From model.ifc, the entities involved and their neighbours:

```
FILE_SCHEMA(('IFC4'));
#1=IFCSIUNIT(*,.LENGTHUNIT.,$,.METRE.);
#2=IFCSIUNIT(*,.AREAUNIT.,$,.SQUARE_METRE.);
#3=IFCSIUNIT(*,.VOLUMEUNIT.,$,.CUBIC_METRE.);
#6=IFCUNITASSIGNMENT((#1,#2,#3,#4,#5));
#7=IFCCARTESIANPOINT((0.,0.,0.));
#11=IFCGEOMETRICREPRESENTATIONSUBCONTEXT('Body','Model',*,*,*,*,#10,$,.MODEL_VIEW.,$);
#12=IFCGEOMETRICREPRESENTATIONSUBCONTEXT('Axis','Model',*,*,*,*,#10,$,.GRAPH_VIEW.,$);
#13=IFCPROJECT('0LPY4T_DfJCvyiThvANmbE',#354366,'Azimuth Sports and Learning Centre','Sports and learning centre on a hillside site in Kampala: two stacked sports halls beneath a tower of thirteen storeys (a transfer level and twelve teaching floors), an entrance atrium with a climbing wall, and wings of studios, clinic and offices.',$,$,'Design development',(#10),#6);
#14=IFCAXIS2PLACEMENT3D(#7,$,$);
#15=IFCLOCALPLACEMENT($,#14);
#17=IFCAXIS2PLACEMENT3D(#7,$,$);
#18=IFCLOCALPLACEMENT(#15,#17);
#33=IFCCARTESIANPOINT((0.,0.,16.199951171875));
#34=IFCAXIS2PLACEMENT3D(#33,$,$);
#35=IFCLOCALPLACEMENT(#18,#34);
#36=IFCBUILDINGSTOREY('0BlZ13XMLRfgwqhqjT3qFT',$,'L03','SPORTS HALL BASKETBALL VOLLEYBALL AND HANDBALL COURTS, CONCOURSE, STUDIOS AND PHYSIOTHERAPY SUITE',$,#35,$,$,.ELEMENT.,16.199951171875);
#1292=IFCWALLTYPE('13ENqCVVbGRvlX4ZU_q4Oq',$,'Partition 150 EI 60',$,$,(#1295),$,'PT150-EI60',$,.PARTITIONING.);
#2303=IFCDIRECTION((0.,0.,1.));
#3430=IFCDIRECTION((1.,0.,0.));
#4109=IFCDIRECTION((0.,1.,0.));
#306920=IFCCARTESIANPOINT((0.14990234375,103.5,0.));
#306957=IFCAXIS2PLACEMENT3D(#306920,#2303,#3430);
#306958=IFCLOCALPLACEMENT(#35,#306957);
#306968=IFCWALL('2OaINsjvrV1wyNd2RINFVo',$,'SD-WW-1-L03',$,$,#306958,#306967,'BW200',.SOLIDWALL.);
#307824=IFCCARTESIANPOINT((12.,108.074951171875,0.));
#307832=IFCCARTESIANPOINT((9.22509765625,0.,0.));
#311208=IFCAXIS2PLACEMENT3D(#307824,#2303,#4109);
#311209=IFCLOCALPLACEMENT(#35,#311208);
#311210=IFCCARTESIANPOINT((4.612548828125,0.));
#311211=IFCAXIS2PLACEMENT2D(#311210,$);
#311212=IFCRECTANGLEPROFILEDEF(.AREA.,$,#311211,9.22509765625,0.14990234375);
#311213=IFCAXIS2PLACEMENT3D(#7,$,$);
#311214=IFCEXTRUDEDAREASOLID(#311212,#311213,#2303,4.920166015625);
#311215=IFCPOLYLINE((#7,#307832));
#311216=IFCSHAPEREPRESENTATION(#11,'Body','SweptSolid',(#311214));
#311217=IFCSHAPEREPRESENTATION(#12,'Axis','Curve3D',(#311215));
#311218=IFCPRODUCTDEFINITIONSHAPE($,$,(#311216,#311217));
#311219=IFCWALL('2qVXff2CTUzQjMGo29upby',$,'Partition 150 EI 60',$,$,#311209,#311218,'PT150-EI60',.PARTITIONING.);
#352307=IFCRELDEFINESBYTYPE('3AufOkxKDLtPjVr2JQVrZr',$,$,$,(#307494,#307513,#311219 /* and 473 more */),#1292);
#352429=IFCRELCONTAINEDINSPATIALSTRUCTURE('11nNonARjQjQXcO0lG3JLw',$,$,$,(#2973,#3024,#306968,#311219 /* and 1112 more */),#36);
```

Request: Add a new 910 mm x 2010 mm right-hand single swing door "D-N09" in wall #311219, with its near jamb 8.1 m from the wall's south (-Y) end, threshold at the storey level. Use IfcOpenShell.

```python
import numpy as np
import ifcopenshell
import ifcopenshell.api.feature
import ifcopenshell.api.geometry
import ifcopenshell.api.root
import ifcopenshell.api.spatial
import ifcopenshell.geom
import ifcopenshell.util.element
import ifcopenshell.util.placement
import ifcopenshell.util.representation
import ifcopenshell.util.shape
import ifcopenshell.util.unit

model = ifcopenshell.open("model.ifc")
unit_scale = ifcopenshell.util.unit.calculate_unit_scale(model)
settings = ifcopenshell.geom.settings()


def volume(element):
    """Net volume in cubic metres, openings subtracted."""
    shape = ifcopenshell.geom.create_shape(settings, element)
    return ifcopenshell.util.shape.get_volume(shape.geometry)


wall = model.by_id(311219)
storey = ifcopenshell.util.element.get_container(wall, ifc_class="IfcBuildingStorey")
context = ifcopenshell.util.representation.get_context(model, "Model", "Body", "MODEL_VIEW")
before = volume(wall)

width, height, from_end, sill = 0.91, 2.01, 8.1, 0.0  # metres

# The wall runs along its own X axis, and the end named is its -X end.
wall_shape = ifcopenshell.geom.create_shape(settings, wall)
x, y, z = ifcopenshell.util.shape.get_vertices(wall_shape.geometry).T
start = x.min() + from_end
face, thickness = float(y.min()), float(y.max() - y.min())
wall_matrix = ifcopenshell.util.placement.get_local_placement(wall.ObjectPlacement)
level = ifcopenshell.util.placement.get_local_placement(storey.ObjectPlacement)[2, 3]


def in_wall(x, y):
    """Placement at x, y metres in the wall's axes, at sill height."""
    matrix = wall_matrix.copy()
    matrix[:, 3] = wall_matrix @ np.array([x / unit_scale, y / unit_scale, 0.0, 1.0])
    matrix[2, 3] = level + sill / unit_scale
    return matrix


# Opening: a box that overshoots both wall faces by 50 mm.
opening = ifcopenshell.api.root.create_entity(model, ifc_class="IfcOpeningElement", predefined_type="OPENING")
box = ifcopenshell.api.geometry.add_wall_representation(
    model, context=context, length=width, height=height, thickness=thickness + 0.1
)
ifcopenshell.api.geometry.assign_representation(model, product=opening, representation=box)
ifcopenshell.api.geometry.edit_object_placement(model, product=opening, matrix=in_wall(start, face - 0.05), is_si=False)
ifcopenshell.api.feature.add_feature(model, feature=opening, element=wall)

door = ifcopenshell.api.root.create_entity(model, ifc_class="IfcDoor", name="D-N09", predefined_type="DOOR")
door.OverallWidth, door.OverallHeight = width / unit_scale, height / unit_scale
door.OperationType = "SINGLE_SWING_RIGHT"
body = ifcopenshell.api.geometry.add_door_representation(
    model,
    context=context,
    overall_width=door.OverallWidth,
    overall_height=door.OverallHeight,
    operation_type="SINGLE_SWING_RIGHT",
    lining_properties={"LiningDepth": thickness / unit_scale, "ThresholdDepth": thickness / unit_scale},
)
ifcopenshell.api.geometry.assign_representation(model, product=door, representation=body)
ifcopenshell.api.spatial.assign_container(model, products=[door], relating_structure=storey)
ifcopenshell.api.feature.add_filling(model, opening=opening, element=door)

# The lining spans the wall, so the door starts at the wall face.
ifcopenshell.api.geometry.edit_object_placement(model, product=door, matrix=in_wall(start, face), is_si=False)

after = volume(wall)

print(f"wall volume {before:.3f} -> {after:.3f} m3")

model.write("model-out.ifc")
```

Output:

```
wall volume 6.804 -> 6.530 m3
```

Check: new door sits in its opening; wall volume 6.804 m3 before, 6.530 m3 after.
